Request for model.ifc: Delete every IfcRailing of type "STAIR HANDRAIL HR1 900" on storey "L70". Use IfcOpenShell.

First a look at what the model holds.

```python
import ifcopenshell
import ifcopenshell.util.element

model = ifcopenshell.open("model.ifc")
print(model.schema)
storey = next(s for s in model.by_type("IfcBuildingStorey") if s.Name == "L70")
railings = [e for e in ifcopenshell.util.element.get_decomposition(storey) if e.is_a("IfcRailing")]
seen = {}
for e in railings:
    element_type = ifcopenshell.util.element.get_type(e)
    name = element_type.Name if element_type not in (None, e) else None
    seen[name] = seen.get(name, 0) + 1
for name, count in sorted(seen.items(), key=str):
    print(count, "x", name)
```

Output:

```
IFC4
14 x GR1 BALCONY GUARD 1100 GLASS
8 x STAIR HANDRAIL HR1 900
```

```python
import ifcopenshell
import ifcopenshell.api.root
import ifcopenshell.util.element

model = ifcopenshell.open("model.ifc")

storey = next(s for s in model.by_type("IfcBuildingStorey") if s.Name == "L70")
railings = [e for e in ifcopenshell.util.element.get_decomposition(storey) if e.is_a("IfcRailing")]
targets = [e for e in railings if (t := ifcopenshell.util.element.get_type(e)) not in (None, e) and t.Name == "STAIR HANDRAIL HR1 900"]

for e in targets:
    ifcopenshell.api.root.remove_product(model, product=e)
print(len(targets), "removed")

model.write("model_updated.ifc")
```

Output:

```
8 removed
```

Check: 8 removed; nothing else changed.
